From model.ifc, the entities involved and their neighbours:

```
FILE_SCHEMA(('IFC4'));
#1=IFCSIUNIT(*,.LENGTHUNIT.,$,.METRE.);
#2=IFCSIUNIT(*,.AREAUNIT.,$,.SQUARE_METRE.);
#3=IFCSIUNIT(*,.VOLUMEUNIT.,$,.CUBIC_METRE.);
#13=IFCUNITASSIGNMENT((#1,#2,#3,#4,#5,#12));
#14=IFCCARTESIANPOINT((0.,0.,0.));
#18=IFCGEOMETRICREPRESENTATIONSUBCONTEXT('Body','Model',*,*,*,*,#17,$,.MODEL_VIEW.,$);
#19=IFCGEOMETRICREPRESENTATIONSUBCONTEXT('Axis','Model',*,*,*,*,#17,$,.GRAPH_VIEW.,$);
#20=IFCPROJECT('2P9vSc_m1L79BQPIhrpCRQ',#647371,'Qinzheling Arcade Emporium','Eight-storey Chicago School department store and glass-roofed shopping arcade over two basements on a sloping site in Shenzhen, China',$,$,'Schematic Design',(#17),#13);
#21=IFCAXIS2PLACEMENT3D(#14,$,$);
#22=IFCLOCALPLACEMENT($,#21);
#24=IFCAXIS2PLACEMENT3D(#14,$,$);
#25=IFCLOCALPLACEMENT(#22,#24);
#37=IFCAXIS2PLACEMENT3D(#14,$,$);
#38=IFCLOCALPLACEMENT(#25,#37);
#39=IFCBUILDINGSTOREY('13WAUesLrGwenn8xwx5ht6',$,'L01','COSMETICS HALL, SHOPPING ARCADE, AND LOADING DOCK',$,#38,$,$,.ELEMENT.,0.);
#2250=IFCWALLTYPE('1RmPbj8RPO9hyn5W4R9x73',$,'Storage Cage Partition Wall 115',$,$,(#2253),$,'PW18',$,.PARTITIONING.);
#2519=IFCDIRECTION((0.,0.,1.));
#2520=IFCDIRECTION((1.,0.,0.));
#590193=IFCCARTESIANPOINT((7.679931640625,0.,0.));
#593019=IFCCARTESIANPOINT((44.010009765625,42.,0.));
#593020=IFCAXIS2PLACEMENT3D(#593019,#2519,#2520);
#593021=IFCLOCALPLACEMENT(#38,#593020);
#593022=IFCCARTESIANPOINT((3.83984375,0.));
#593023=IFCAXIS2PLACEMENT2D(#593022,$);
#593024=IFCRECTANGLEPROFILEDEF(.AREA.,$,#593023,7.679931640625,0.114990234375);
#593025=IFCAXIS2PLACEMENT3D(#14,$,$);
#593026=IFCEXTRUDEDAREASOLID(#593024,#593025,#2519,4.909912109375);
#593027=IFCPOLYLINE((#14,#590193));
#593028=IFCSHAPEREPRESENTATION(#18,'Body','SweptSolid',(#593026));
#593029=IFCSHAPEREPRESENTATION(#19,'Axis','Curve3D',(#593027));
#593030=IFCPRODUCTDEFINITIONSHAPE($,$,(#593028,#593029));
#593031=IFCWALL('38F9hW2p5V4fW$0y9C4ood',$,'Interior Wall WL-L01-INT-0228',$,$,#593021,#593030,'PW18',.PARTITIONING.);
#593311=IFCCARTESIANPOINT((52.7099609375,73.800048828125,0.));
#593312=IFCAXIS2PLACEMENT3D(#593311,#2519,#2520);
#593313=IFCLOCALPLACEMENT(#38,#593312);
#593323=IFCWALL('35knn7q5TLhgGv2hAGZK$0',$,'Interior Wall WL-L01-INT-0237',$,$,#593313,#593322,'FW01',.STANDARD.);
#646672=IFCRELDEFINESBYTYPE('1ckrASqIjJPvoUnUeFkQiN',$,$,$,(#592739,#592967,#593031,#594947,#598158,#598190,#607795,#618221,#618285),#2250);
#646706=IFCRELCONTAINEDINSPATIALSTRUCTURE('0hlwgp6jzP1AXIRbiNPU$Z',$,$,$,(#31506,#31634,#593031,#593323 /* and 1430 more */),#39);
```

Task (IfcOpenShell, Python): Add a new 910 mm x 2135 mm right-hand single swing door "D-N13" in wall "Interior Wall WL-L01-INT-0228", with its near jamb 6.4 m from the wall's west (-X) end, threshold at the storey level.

```python
import numpy as np
import ifcopenshell
import ifcopenshell.api.feature
import ifcopenshell.api.geometry
import ifcopenshell.api.root
import ifcopenshell.api.spatial
import ifcopenshell.geom
import ifcopenshell.util.element
import ifcopenshell.util.placement
import ifcopenshell.util.representation
import ifcopenshell.util.shape
import ifcopenshell.util.unit

model = ifcopenshell.open("model.ifc")
unit_scale = ifcopenshell.util.unit.calculate_unit_scale(model)
settings = ifcopenshell.geom.settings()


def volume(element):
    """Net volume in cubic metres, openings subtracted."""
    shape = ifcopenshell.geom.create_shape(settings, element)
    return ifcopenshell.util.shape.get_volume(shape.geometry)


wall = model.by_guid("38F9hW2p5V4fW$0y9C4ood")
storey = ifcopenshell.util.element.get_container(wall, ifc_class="IfcBuildingStorey")
context = ifcopenshell.util.representation.get_context(model, "Model", "Body", "MODEL_VIEW")
before = volume(wall)

width, height, from_end, sill = 0.91, 2.135, 6.4, 0.0  # metres

# The wall runs along its own X axis, and the end named is its -X end.
wall_shape = ifcopenshell.geom.create_shape(settings, wall)
x, y, z = ifcopenshell.util.shape.get_vertices(wall_shape.geometry).T
start = x.min() + from_end
face, thickness = float(y.min()), float(y.max() - y.min())
wall_matrix = ifcopenshell.util.placement.get_local_placement(wall.ObjectPlacement)
level = ifcopenshell.util.placement.get_local_placement(storey.ObjectPlacement)[2, 3]


def in_wall(x, y):
    """Placement at x, y metres in the wall's axes, at sill height."""
    matrix = wall_matrix.copy()
    matrix[:, 3] = wall_matrix @ np.array([x / unit_scale, y / unit_scale, 0.0, 1.0])
    matrix[2, 3] = level + sill / unit_scale
    return matrix


# Opening: a box that overshoots both wall faces by 50 mm.
opening = ifcopenshell.api.root.create_entity(model, ifc_class="IfcOpeningElement", predefined_type="OPENING")
box = ifcopenshell.api.geometry.add_wall_representation(
    model, context=context, length=width, height=height, thickness=thickness + 0.1
)
ifcopenshell.api.geometry.assign_representation(model, product=opening, representation=box)
ifcopenshell.api.geometry.edit_object_placement(model, product=opening, matrix=in_wall(start, face - 0.05), is_si=False)
ifcopenshell.api.feature.add_feature(model, feature=opening, element=wall)

door = ifcopenshell.api.root.create_entity(model, ifc_class="IfcDoor", name="D-N13", predefined_type="DOOR")
door.OverallWidth, door.OverallHeight = width / unit_scale, height / unit_scale
door.OperationType = "SINGLE_SWING_RIGHT"
body = ifcopenshell.api.geometry.add_door_representation(
    model,
    context=context,
    overall_width=door.OverallWidth,
    overall_height=door.OverallHeight,
    operation_type="SINGLE_SWING_RIGHT",
    lining_properties={"LiningDepth": thickness / unit_scale, "ThresholdDepth": thickness / unit_scale},
)
ifcopenshell.api.geometry.assign_representation(model, product=door, representation=body)
ifcopenshell.api.spatial.assign_container(model, products=[door], relating_structure=storey)
ifcopenshell.api.feature.add_filling(model, opening=opening, element=door)

# The lining spans the wall, so the door starts at the wall face.
ifcopenshell.api.geometry.edit_object_placement(model, product=door, matrix=in_wall(start, face), is_si=False)

after = volume(wall)

print(f"wall volume {before:.3f} -> {after:.3f} m3")

model.write("model_edited.ifc")
```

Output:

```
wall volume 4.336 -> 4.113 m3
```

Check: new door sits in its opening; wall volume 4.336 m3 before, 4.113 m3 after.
